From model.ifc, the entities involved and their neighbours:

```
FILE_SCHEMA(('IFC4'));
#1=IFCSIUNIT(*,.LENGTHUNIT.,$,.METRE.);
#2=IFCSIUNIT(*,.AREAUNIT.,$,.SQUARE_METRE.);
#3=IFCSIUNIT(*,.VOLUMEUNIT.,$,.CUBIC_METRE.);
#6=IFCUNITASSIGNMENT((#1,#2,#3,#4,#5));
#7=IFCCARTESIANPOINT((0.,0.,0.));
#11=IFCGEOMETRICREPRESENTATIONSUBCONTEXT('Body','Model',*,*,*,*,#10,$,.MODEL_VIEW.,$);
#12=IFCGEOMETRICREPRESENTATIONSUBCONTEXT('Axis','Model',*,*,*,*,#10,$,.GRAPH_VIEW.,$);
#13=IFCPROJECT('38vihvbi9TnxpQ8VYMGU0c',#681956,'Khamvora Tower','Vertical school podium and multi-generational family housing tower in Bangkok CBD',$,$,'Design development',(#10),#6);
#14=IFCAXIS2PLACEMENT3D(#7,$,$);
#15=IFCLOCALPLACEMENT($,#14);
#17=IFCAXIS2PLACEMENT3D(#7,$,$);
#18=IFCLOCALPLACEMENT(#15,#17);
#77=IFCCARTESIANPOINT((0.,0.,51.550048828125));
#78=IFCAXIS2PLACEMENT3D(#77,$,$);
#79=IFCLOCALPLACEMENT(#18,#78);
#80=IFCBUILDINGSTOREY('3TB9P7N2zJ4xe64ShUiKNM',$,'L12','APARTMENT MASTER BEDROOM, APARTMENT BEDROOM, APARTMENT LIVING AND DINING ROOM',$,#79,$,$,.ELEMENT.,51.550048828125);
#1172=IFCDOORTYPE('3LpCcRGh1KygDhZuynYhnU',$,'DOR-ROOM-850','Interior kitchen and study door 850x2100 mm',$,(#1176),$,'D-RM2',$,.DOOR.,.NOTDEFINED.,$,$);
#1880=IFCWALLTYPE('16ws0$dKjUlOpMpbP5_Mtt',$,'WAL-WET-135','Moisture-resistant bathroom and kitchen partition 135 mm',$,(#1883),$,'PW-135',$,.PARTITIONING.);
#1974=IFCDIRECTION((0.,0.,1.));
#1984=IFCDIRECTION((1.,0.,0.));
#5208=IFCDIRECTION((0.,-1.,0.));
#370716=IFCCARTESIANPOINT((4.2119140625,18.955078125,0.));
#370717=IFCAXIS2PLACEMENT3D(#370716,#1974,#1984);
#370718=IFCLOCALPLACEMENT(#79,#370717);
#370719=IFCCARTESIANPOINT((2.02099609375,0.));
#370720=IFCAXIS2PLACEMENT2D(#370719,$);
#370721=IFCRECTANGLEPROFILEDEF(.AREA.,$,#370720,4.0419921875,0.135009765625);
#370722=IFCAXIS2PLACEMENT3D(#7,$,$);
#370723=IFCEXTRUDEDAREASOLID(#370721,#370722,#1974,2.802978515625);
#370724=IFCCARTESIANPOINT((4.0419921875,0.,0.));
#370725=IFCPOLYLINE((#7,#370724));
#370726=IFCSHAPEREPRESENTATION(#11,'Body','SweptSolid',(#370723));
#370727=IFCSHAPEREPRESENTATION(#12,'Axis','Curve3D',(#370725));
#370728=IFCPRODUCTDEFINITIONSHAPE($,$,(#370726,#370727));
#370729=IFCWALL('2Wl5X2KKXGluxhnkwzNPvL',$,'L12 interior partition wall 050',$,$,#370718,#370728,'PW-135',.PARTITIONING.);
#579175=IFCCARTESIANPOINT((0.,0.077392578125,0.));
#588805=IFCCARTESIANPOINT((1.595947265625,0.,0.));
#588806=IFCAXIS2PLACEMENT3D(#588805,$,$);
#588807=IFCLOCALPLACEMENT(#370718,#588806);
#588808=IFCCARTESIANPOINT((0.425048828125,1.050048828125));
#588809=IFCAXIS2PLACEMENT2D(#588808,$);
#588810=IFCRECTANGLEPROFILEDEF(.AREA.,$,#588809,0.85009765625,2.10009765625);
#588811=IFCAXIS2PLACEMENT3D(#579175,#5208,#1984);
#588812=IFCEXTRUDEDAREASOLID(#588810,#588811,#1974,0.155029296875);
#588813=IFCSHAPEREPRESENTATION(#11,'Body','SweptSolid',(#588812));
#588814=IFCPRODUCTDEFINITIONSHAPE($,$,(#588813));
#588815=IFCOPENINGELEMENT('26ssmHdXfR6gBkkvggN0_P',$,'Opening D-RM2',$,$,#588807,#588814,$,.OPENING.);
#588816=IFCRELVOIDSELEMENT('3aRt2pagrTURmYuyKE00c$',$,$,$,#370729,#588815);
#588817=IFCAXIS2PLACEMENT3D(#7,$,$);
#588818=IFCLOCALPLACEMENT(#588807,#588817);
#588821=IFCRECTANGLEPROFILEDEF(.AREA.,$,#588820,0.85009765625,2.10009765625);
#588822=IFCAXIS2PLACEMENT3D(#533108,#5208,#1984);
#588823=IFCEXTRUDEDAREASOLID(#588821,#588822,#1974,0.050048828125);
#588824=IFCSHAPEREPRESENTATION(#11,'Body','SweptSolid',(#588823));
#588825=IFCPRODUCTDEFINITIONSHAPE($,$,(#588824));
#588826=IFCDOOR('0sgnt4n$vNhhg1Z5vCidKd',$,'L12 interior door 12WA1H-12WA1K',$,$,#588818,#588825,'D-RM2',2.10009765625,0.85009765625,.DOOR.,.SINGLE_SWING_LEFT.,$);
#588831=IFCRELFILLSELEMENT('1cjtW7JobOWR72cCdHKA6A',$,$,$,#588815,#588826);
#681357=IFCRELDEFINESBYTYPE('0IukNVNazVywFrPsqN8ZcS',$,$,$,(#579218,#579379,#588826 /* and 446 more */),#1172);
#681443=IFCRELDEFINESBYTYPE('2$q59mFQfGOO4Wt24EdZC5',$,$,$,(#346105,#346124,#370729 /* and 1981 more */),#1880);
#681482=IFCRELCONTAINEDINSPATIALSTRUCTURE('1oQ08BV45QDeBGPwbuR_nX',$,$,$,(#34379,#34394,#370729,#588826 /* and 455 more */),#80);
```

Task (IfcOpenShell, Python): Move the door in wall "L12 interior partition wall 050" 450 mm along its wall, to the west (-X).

```python
import ifcopenshell
import ifcopenshell.api.geometry
import ifcopenshell.util.placement
import ifcopenshell.util.unit

model = ifcopenshell.open("model.ifc")
unit_scale = ifcopenshell.util.unit.calculate_unit_scale(model)

door = model.by_guid("0sgnt4n$vNhhg1Z5vCidKd")
opening = door.FillsVoids[0].RelatingOpeningElement
wall = opening.VoidsElements[0].RelatingBuildingElement

wall_matrix = ifcopenshell.util.placement.get_local_placement(wall.ObjectPlacement)
shift = wall_matrix[:3, 0] * -0.45 / unit_scale
before = ifcopenshell.util.placement.get_local_placement(door.ObjectPlacement)[:3, 3].copy()

# The door is placed relative to its opening, so it follows when the opening moves.
matrix = ifcopenshell.util.placement.get_local_placement(opening.ObjectPlacement)
matrix[:3, 3] += shift
ifcopenshell.api.geometry.edit_object_placement(
    model, product=opening, matrix=matrix, is_si=False, should_transform_children=True
)

after = ifcopenshell.util.placement.get_local_placement(door.ObjectPlacement)[:3, 3]
print("door moved by", (after - before).round(3) + 0.0)

model.write("model_edited.ifc")
```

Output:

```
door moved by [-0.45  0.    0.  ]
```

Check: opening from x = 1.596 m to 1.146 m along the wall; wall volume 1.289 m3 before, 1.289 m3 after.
